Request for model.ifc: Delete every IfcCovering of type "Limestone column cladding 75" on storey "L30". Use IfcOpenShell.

First a look at what the model holds.

```python
import ifcopenshell
import ifcopenshell.util.element

model = ifcopenshell.open("model.ifc")
print(model.schema)
storey = next(s for s in model.by_type("IfcBuildingStorey") if s.Name == "L30")
coverings = [e for e in ifcopenshell.util.element.get_decomposition(storey) if e.is_a("IfcCovering")]
seen = {}
for e in coverings:
    element_type = ifcopenshell.util.element.get_type(e)
    name = element_type.Name if element_type not in (None, e) else None
    seen[name] = seen.get(name, 0) + 1
for name, count in sorted(seen.items(), key=str):
    print(count, "x", name)
```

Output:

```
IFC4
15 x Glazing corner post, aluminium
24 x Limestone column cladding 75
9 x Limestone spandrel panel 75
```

```python
import ifcopenshell
import ifcopenshell.api.root
import ifcopenshell.util.element

model = ifcopenshell.open("model.ifc")

storey = next(s for s in model.by_type("IfcBuildingStorey") if s.Name == "L30")
coverings = [e for e in ifcopenshell.util.element.get_decomposition(storey) if e.is_a("IfcCovering")]
targets = [e for e in coverings if (t := ifcopenshell.util.element.get_type(e)) not in (None, e) and t.Name == "Limestone column cladding 75"]

for e in targets:
    ifcopenshell.api.root.remove_product(model, product=e)
print(len(targets), "removed")

model.write("model_v2.ifc")
```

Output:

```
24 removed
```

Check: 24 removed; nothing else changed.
